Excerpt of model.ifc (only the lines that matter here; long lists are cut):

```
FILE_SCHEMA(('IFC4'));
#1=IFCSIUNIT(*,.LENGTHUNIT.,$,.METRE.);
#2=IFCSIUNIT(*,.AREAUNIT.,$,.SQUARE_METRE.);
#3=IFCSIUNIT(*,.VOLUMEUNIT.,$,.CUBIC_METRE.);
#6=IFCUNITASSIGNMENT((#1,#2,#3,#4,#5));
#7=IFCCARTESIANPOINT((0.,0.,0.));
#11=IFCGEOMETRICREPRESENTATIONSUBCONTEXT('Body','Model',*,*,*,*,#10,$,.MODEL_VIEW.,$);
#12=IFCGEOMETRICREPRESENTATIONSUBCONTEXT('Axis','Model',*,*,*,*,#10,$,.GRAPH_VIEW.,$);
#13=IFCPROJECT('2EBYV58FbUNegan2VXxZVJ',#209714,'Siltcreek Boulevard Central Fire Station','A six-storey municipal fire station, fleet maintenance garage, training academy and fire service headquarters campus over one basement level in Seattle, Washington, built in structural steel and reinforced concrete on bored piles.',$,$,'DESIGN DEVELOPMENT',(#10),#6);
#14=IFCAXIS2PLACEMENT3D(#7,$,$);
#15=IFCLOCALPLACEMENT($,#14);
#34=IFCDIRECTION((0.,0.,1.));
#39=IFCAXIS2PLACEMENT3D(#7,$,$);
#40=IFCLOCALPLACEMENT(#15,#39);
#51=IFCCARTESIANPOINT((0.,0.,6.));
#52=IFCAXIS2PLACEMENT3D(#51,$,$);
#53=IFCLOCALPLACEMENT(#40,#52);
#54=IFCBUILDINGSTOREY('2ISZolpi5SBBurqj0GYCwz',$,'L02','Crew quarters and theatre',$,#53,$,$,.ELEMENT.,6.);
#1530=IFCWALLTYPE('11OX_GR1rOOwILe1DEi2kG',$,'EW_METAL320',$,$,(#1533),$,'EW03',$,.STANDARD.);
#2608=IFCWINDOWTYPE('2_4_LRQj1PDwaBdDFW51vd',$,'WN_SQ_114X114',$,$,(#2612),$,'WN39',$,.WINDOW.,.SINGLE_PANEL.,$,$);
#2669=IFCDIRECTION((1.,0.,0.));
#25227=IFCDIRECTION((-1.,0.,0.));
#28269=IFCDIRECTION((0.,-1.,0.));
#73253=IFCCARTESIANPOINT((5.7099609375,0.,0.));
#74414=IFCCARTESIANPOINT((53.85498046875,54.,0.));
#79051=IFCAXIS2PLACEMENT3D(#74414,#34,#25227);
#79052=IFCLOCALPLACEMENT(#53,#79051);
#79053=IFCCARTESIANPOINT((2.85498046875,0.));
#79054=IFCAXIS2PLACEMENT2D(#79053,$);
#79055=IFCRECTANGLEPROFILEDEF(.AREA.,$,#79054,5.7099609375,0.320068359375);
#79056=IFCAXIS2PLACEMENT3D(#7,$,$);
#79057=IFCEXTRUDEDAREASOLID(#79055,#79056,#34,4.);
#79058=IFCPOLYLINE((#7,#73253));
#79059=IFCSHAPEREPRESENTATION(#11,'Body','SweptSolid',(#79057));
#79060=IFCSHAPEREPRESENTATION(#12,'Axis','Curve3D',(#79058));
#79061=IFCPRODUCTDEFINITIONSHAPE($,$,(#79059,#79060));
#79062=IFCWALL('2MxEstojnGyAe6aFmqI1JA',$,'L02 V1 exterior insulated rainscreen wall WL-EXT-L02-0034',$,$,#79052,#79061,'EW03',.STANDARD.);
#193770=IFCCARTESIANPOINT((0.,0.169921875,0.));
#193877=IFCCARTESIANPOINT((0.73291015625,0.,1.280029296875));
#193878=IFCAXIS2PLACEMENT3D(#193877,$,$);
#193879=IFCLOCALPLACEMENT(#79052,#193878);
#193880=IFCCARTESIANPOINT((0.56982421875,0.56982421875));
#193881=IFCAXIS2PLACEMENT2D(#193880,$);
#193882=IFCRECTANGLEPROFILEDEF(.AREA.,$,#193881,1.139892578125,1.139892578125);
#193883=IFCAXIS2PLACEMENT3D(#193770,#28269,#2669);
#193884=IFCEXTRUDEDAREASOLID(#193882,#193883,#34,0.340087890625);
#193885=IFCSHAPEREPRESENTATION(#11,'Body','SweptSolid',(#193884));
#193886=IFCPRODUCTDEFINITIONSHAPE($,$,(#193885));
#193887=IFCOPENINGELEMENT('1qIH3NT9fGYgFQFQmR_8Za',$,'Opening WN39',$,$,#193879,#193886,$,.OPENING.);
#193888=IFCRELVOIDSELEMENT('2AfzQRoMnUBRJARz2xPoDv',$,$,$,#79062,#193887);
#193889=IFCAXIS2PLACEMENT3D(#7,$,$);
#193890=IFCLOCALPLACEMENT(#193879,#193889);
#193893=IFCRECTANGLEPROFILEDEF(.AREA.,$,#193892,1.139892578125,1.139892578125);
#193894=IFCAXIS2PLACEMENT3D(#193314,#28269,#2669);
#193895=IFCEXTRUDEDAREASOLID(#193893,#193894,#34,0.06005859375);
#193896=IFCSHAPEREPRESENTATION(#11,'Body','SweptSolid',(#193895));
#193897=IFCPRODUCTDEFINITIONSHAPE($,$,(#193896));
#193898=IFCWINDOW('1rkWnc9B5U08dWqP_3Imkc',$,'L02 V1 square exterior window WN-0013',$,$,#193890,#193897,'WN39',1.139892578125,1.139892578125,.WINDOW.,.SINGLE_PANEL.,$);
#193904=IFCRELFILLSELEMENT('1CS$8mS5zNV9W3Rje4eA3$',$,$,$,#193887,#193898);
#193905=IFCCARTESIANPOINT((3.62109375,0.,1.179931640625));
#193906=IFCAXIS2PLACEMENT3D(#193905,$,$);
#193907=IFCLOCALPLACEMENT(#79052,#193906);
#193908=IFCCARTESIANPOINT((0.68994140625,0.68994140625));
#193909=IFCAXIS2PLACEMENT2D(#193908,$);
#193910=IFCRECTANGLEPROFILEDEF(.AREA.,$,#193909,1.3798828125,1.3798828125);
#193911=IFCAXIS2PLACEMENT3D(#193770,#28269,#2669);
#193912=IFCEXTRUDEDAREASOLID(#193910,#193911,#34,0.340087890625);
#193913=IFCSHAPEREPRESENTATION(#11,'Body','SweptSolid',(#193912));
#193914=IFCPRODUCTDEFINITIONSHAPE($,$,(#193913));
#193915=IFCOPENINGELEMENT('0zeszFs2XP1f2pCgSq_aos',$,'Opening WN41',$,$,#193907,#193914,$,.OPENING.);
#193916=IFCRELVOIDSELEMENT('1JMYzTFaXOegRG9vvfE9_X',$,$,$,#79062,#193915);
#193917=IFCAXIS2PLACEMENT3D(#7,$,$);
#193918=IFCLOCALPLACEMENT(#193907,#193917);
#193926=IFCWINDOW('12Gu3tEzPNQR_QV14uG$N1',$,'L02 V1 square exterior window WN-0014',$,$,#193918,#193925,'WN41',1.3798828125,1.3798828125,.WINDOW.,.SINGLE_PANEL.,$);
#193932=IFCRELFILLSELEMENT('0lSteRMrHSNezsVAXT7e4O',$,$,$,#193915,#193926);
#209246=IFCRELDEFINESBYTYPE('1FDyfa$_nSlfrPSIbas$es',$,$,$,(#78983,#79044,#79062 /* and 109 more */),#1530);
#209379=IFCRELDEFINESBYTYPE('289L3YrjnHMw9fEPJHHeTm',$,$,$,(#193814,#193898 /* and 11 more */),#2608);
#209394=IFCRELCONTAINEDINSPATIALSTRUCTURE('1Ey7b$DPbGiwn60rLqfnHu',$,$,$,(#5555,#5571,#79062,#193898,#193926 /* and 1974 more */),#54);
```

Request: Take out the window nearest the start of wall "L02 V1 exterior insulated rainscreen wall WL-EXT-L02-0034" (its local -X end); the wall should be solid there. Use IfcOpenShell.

```python
import ifcopenshell
import ifcopenshell.api.feature
import ifcopenshell.api.root
import ifcopenshell.geom
import ifcopenshell.util.shape

model = ifcopenshell.open("model.ifc")
settings = ifcopenshell.geom.settings()


def volume(element):
    """Net volume in cubic metres, openings subtracted."""
    shape = ifcopenshell.geom.create_shape(settings, element)
    return ifcopenshell.util.shape.get_volume(shape.geometry)


window = model.by_guid("1rkWnc9B5U08dWqP_3Imkc")
opening = window.FillsVoids[0].RelatingOpeningElement
wall = opening.VoidsElements[0].RelatingBuildingElement
before = volume(wall)

ifcopenshell.api.root.remove_product(model, product=window)
ifcopenshell.api.feature.remove_feature(model, feature=opening)

after = volume(wall)

print(f"wall volume {before:.3f} -> {after:.3f} m3")

model.write("model_edited.ifc")
```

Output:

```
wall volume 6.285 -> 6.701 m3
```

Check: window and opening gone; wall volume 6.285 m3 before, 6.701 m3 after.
